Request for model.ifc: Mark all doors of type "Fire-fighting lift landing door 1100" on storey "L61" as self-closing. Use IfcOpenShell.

First a look at what the model holds.

```python
import ifcopenshell
import ifcopenshell.util.element

model = ifcopenshell.open("model.ifc")
print(model.schema)
storey = next(s for s in model.by_type("IfcBuildingStorey") if s.Name == "L61")
doors = [e for e in ifcopenshell.util.element.get_decomposition(storey) if e.is_a("IfcDoor")]
seen = {}
for e in doors:
    element_type = ifcopenshell.util.element.get_type(e)
    key = (element_type.Name if element_type != e and element_type else None, ifcopenshell.util.element.get_pset(e, "Pset_DoorCommon", "SelfClosing"))
    seen[key] = seen.get(key, 0) + 1
for (name, value), count in sorted(seen.items(), key=str):
    print(count, "x", name, "|", value)
```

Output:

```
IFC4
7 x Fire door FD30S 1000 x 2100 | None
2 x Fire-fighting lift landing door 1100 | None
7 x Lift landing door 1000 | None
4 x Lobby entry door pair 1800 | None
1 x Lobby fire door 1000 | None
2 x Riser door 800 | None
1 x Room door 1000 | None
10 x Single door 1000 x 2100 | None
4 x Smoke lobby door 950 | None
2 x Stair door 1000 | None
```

```python
import ifcopenshell
import ifcopenshell.api.pset
import ifcopenshell.util.element

model = ifcopenshell.open("model.ifc")

storey = next(s for s in model.by_type("IfcBuildingStorey") if s.Name == "L61")
doors = [e for e in ifcopenshell.util.element.get_decomposition(storey) if e.is_a("IfcDoor")]

count = 0
for e in doors:
    element_type = ifcopenshell.util.element.get_type(e)
    if element_type in (None, e) or element_type.Name != "Fire-fighting lift landing door 1100":
        continue
    # add_pset returns the element's existing set when there is one.
    pset = ifcopenshell.api.pset.add_pset(model, product=e, name="Pset_DoorCommon")
    ifcopenshell.api.pset.edit_pset(model, pset=pset, properties={"SelfClosing": True})
    count += 1

print(count, "doors updated")

model.write("model_rev.ifc")
```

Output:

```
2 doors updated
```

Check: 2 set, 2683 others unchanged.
